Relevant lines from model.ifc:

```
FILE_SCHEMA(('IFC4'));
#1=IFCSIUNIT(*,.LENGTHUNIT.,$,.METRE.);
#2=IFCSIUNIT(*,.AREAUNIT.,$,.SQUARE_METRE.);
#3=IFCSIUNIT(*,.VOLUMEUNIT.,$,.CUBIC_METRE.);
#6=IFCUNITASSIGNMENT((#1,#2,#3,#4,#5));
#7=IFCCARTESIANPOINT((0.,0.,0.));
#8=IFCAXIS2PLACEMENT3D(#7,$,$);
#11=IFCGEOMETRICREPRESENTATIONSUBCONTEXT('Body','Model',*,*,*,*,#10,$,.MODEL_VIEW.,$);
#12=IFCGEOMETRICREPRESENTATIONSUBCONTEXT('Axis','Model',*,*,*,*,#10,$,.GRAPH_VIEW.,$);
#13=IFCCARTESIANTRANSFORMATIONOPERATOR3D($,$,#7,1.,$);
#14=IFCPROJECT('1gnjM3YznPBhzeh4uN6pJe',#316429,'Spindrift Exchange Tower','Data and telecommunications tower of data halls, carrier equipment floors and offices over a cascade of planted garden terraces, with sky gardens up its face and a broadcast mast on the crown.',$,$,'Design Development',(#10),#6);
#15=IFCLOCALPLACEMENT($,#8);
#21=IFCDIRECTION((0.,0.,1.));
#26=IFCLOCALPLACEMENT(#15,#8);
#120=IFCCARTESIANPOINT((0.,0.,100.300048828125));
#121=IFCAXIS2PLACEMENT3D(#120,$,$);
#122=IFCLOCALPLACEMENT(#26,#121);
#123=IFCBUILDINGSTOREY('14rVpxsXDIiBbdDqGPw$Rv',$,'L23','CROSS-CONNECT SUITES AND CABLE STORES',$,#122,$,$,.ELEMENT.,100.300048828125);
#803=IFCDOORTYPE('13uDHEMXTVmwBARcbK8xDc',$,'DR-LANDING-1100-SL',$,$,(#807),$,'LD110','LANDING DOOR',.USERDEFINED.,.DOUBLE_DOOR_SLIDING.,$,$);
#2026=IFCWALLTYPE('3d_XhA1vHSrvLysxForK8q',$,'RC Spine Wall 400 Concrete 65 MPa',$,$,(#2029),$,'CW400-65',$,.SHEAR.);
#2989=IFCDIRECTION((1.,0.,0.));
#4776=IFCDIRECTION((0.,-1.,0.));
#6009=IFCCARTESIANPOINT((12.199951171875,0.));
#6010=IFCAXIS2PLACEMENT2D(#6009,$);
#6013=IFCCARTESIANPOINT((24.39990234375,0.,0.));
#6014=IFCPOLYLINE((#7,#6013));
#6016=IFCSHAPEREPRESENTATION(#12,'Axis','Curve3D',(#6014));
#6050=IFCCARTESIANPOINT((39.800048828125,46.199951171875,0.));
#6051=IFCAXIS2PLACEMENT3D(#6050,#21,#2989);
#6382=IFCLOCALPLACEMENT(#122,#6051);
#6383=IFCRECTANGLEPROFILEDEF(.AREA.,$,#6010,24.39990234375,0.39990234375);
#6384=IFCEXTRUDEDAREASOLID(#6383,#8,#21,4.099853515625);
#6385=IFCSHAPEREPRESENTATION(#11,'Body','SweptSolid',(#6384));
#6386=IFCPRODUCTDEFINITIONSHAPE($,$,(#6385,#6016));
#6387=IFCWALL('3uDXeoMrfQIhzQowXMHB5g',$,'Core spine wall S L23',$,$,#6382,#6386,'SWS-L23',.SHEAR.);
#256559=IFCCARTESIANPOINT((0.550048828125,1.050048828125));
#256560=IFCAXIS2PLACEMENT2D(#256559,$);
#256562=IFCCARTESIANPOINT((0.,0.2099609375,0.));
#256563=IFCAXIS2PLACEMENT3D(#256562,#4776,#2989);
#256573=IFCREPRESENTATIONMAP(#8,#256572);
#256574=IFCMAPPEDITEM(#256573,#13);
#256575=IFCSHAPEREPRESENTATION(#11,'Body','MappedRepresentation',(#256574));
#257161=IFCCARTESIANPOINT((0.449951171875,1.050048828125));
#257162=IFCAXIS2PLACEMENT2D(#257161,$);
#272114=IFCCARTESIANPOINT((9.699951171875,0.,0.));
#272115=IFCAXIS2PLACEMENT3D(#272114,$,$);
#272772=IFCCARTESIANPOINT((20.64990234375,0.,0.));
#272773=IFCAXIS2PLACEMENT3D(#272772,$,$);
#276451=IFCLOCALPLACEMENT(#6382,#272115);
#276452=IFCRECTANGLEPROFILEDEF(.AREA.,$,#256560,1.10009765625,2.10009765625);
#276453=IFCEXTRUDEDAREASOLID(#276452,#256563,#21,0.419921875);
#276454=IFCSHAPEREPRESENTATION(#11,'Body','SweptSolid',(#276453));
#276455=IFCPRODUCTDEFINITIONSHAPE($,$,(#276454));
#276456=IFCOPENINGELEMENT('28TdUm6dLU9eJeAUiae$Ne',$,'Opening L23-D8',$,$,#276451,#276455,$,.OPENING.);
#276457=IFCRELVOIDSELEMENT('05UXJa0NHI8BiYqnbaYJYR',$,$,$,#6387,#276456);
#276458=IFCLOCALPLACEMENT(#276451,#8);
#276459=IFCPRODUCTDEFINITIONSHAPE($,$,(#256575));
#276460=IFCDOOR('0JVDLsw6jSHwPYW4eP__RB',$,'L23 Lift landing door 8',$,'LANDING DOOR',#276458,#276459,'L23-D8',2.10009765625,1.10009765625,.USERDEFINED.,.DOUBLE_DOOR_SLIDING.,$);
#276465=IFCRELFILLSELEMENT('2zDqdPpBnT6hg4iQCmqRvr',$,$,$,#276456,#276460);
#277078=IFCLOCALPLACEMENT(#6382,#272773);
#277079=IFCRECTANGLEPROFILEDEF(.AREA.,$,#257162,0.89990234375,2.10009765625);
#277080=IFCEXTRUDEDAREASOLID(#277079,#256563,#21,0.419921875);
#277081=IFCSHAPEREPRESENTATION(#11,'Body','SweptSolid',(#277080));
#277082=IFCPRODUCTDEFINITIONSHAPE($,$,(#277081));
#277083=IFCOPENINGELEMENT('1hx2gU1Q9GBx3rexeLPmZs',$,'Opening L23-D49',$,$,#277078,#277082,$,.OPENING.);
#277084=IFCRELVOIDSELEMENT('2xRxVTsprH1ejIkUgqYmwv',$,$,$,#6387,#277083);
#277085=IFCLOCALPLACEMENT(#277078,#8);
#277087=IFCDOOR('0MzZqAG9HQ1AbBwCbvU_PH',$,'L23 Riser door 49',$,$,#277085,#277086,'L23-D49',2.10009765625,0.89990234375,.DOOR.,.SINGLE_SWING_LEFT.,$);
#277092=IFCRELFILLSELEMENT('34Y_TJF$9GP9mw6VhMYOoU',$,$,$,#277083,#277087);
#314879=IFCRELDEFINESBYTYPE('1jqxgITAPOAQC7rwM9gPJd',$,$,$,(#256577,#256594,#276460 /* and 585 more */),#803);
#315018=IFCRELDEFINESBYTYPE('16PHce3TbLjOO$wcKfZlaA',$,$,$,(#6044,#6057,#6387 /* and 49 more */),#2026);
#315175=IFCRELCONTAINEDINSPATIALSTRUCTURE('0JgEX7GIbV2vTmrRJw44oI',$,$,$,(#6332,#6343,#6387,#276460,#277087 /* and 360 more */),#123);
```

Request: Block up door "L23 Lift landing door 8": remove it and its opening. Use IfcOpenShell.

```python
import ifcopenshell
import ifcopenshell.api.feature
import ifcopenshell.api.root
import ifcopenshell.geom
import ifcopenshell.util.shape

model = ifcopenshell.open("model.ifc")
settings = ifcopenshell.geom.settings()


def volume(element):
    """Net volume in cubic metres, openings subtracted."""
    shape = ifcopenshell.geom.create_shape(settings, element)
    return ifcopenshell.util.shape.get_volume(shape.geometry)


door = model.by_id(276460)
opening = door.FillsVoids[0].RelatingOpeningElement
wall = opening.VoidsElements[0].RelatingBuildingElement
before = volume(wall)

ifcopenshell.api.root.remove_product(model, product=door)
ifcopenshell.api.feature.remove_feature(model, feature=opening)

after = volume(wall)

print(f"wall volume {before:.3f} -> {after:.3f} m3")

model.write("model_rev.ifc")
```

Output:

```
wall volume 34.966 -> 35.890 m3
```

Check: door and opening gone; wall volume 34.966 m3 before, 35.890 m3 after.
